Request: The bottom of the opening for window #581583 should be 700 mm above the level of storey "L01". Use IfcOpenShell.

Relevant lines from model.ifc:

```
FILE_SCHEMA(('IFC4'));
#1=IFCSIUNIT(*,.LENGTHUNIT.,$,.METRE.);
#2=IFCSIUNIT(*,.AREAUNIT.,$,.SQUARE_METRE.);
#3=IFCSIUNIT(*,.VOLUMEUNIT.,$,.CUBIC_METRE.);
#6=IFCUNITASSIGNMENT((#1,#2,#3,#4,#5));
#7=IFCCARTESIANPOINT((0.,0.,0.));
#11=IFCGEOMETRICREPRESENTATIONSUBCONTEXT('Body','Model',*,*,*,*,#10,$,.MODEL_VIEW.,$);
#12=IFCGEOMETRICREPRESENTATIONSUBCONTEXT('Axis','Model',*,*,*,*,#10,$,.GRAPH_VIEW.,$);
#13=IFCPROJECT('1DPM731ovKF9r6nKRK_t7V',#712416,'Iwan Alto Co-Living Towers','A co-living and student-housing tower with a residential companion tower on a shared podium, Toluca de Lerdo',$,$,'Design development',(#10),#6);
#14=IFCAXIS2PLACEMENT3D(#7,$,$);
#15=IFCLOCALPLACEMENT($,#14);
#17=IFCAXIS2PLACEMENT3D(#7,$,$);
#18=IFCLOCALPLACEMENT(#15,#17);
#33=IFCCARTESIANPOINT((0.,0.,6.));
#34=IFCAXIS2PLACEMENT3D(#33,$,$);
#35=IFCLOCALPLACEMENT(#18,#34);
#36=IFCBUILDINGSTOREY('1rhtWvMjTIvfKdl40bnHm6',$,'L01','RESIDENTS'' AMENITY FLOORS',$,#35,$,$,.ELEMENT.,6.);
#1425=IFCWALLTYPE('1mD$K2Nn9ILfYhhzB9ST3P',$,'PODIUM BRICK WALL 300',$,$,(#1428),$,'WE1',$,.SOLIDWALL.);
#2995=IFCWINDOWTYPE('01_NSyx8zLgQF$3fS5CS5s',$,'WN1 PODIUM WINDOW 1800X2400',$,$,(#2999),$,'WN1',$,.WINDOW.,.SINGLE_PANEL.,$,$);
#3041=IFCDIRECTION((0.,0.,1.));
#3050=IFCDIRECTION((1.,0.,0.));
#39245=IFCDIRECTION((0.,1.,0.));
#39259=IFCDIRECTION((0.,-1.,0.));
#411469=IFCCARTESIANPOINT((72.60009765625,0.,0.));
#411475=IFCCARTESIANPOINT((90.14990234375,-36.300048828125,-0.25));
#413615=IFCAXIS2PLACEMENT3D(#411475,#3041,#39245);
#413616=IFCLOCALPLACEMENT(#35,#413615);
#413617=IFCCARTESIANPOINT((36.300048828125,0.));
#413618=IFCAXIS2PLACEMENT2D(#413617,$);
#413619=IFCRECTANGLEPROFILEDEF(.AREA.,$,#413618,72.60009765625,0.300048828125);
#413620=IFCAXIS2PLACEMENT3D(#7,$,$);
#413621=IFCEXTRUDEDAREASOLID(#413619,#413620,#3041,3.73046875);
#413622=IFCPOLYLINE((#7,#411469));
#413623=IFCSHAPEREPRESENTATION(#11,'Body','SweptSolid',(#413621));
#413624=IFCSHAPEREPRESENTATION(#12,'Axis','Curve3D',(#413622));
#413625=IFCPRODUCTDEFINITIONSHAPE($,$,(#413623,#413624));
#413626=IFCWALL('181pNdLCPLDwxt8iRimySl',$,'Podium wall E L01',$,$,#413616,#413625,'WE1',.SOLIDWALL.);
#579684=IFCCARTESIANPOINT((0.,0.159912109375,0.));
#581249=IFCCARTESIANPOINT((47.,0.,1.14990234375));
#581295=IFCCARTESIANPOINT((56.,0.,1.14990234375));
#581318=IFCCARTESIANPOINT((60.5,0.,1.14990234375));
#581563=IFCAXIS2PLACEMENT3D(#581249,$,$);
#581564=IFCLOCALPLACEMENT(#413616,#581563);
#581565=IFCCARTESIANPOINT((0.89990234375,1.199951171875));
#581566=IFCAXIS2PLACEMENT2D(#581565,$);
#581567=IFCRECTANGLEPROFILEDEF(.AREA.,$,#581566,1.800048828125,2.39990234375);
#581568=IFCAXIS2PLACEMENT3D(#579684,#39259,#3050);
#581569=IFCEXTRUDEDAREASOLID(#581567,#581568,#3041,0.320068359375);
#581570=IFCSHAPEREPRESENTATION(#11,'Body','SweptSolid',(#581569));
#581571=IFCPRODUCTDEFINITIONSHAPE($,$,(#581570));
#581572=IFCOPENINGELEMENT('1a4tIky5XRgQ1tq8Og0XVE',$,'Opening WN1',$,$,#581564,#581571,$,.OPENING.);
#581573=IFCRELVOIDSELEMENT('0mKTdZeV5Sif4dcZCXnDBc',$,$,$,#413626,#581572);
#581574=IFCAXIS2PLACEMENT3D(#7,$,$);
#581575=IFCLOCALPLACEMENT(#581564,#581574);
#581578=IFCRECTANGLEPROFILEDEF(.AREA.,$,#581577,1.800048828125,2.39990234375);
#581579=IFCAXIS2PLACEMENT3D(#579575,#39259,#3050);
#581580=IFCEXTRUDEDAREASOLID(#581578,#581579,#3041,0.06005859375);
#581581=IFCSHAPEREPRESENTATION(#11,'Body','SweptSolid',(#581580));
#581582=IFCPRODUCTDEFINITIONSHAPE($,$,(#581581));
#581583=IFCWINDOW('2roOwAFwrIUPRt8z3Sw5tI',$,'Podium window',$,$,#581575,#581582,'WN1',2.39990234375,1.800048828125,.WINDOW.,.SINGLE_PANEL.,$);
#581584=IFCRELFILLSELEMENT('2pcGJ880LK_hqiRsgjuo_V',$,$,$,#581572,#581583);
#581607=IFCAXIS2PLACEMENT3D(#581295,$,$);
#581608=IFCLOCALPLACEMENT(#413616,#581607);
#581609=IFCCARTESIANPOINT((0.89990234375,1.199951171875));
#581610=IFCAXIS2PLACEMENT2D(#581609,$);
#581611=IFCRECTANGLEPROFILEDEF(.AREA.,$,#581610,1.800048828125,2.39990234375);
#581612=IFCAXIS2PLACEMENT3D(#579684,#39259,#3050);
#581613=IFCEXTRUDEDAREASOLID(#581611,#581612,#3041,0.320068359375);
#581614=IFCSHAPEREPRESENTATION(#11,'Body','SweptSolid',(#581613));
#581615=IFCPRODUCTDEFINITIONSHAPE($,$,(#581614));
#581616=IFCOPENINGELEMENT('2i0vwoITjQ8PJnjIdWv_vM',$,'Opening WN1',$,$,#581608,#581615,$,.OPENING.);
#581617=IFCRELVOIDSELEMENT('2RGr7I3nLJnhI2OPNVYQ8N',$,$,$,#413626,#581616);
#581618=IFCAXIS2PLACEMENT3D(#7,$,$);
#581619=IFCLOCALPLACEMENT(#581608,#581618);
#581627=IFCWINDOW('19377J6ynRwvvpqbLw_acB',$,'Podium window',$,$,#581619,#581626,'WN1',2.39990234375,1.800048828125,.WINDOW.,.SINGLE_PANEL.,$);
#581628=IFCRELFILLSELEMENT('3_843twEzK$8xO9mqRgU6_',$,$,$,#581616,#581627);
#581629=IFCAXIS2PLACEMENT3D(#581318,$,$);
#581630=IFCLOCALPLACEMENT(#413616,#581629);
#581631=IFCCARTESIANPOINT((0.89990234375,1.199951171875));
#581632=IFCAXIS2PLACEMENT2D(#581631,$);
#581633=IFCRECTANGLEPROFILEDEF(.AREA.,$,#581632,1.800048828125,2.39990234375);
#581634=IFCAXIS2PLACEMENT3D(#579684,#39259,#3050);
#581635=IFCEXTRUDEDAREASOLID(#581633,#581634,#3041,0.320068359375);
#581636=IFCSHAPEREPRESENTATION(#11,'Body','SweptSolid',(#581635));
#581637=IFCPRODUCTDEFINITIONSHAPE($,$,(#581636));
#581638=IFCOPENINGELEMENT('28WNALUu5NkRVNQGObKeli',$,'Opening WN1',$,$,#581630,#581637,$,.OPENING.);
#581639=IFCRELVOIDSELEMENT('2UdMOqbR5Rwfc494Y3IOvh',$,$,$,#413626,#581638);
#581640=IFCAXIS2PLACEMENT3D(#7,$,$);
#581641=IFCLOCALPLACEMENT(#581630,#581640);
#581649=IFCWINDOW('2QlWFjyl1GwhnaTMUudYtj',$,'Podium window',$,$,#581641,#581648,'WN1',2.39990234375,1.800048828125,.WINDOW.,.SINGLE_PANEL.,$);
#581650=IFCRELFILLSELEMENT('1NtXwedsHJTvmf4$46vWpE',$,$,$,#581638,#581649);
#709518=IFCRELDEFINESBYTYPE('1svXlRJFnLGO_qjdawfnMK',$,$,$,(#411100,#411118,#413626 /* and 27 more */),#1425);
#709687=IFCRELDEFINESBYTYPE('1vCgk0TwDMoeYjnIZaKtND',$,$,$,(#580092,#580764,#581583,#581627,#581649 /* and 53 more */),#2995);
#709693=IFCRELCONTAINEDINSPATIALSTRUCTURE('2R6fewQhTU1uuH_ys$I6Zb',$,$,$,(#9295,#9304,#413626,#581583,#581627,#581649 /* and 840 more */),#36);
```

```python
import numpy as np
import ifcopenshell
import ifcopenshell.api.geometry
import ifcopenshell.geom
import ifcopenshell.util.element
import ifcopenshell.util.placement
import ifcopenshell.util.shape
import ifcopenshell.util.unit

model = ifcopenshell.open("model.ifc")
unit_scale = ifcopenshell.util.unit.calculate_unit_scale(model)

window = model.by_guid("2roOwAFwrIUPRt8z3Sw5tI")
opening = window.FillsVoids[0].RelatingOpeningElement
storey = ifcopenshell.util.element.get_container(window, ifc_class="IfcBuildingStorey")
level = ifcopenshell.util.placement.get_local_placement(storey.ObjectPlacement)[2, 3]

# The opening's origin need not be at the sill, so measure its lowest point.
shape = ifcopenshell.geom.create_shape(ifcopenshell.geom.settings(), opening)
bottom = ifcopenshell.util.shape.get_shape_bottom_elevation(shape, shape.geometry) / unit_scale
dz = level + 0.7 / unit_scale - bottom

shift = np.array([0.0, 0.0, dz])
# The window is placed relative to its opening, so it follows when the opening moves.
matrix = ifcopenshell.util.placement.get_local_placement(opening.ObjectPlacement)
matrix[:3, 3] += shift
ifcopenshell.api.geometry.edit_object_placement(
    model, product=opening, matrix=matrix, is_si=False, should_transform_children=True
)

print(f"moved by {dz * unit_scale:+.3f} m")

model.write("model_updated.ifc")
```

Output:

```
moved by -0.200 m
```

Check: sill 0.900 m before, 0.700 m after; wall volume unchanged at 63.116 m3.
